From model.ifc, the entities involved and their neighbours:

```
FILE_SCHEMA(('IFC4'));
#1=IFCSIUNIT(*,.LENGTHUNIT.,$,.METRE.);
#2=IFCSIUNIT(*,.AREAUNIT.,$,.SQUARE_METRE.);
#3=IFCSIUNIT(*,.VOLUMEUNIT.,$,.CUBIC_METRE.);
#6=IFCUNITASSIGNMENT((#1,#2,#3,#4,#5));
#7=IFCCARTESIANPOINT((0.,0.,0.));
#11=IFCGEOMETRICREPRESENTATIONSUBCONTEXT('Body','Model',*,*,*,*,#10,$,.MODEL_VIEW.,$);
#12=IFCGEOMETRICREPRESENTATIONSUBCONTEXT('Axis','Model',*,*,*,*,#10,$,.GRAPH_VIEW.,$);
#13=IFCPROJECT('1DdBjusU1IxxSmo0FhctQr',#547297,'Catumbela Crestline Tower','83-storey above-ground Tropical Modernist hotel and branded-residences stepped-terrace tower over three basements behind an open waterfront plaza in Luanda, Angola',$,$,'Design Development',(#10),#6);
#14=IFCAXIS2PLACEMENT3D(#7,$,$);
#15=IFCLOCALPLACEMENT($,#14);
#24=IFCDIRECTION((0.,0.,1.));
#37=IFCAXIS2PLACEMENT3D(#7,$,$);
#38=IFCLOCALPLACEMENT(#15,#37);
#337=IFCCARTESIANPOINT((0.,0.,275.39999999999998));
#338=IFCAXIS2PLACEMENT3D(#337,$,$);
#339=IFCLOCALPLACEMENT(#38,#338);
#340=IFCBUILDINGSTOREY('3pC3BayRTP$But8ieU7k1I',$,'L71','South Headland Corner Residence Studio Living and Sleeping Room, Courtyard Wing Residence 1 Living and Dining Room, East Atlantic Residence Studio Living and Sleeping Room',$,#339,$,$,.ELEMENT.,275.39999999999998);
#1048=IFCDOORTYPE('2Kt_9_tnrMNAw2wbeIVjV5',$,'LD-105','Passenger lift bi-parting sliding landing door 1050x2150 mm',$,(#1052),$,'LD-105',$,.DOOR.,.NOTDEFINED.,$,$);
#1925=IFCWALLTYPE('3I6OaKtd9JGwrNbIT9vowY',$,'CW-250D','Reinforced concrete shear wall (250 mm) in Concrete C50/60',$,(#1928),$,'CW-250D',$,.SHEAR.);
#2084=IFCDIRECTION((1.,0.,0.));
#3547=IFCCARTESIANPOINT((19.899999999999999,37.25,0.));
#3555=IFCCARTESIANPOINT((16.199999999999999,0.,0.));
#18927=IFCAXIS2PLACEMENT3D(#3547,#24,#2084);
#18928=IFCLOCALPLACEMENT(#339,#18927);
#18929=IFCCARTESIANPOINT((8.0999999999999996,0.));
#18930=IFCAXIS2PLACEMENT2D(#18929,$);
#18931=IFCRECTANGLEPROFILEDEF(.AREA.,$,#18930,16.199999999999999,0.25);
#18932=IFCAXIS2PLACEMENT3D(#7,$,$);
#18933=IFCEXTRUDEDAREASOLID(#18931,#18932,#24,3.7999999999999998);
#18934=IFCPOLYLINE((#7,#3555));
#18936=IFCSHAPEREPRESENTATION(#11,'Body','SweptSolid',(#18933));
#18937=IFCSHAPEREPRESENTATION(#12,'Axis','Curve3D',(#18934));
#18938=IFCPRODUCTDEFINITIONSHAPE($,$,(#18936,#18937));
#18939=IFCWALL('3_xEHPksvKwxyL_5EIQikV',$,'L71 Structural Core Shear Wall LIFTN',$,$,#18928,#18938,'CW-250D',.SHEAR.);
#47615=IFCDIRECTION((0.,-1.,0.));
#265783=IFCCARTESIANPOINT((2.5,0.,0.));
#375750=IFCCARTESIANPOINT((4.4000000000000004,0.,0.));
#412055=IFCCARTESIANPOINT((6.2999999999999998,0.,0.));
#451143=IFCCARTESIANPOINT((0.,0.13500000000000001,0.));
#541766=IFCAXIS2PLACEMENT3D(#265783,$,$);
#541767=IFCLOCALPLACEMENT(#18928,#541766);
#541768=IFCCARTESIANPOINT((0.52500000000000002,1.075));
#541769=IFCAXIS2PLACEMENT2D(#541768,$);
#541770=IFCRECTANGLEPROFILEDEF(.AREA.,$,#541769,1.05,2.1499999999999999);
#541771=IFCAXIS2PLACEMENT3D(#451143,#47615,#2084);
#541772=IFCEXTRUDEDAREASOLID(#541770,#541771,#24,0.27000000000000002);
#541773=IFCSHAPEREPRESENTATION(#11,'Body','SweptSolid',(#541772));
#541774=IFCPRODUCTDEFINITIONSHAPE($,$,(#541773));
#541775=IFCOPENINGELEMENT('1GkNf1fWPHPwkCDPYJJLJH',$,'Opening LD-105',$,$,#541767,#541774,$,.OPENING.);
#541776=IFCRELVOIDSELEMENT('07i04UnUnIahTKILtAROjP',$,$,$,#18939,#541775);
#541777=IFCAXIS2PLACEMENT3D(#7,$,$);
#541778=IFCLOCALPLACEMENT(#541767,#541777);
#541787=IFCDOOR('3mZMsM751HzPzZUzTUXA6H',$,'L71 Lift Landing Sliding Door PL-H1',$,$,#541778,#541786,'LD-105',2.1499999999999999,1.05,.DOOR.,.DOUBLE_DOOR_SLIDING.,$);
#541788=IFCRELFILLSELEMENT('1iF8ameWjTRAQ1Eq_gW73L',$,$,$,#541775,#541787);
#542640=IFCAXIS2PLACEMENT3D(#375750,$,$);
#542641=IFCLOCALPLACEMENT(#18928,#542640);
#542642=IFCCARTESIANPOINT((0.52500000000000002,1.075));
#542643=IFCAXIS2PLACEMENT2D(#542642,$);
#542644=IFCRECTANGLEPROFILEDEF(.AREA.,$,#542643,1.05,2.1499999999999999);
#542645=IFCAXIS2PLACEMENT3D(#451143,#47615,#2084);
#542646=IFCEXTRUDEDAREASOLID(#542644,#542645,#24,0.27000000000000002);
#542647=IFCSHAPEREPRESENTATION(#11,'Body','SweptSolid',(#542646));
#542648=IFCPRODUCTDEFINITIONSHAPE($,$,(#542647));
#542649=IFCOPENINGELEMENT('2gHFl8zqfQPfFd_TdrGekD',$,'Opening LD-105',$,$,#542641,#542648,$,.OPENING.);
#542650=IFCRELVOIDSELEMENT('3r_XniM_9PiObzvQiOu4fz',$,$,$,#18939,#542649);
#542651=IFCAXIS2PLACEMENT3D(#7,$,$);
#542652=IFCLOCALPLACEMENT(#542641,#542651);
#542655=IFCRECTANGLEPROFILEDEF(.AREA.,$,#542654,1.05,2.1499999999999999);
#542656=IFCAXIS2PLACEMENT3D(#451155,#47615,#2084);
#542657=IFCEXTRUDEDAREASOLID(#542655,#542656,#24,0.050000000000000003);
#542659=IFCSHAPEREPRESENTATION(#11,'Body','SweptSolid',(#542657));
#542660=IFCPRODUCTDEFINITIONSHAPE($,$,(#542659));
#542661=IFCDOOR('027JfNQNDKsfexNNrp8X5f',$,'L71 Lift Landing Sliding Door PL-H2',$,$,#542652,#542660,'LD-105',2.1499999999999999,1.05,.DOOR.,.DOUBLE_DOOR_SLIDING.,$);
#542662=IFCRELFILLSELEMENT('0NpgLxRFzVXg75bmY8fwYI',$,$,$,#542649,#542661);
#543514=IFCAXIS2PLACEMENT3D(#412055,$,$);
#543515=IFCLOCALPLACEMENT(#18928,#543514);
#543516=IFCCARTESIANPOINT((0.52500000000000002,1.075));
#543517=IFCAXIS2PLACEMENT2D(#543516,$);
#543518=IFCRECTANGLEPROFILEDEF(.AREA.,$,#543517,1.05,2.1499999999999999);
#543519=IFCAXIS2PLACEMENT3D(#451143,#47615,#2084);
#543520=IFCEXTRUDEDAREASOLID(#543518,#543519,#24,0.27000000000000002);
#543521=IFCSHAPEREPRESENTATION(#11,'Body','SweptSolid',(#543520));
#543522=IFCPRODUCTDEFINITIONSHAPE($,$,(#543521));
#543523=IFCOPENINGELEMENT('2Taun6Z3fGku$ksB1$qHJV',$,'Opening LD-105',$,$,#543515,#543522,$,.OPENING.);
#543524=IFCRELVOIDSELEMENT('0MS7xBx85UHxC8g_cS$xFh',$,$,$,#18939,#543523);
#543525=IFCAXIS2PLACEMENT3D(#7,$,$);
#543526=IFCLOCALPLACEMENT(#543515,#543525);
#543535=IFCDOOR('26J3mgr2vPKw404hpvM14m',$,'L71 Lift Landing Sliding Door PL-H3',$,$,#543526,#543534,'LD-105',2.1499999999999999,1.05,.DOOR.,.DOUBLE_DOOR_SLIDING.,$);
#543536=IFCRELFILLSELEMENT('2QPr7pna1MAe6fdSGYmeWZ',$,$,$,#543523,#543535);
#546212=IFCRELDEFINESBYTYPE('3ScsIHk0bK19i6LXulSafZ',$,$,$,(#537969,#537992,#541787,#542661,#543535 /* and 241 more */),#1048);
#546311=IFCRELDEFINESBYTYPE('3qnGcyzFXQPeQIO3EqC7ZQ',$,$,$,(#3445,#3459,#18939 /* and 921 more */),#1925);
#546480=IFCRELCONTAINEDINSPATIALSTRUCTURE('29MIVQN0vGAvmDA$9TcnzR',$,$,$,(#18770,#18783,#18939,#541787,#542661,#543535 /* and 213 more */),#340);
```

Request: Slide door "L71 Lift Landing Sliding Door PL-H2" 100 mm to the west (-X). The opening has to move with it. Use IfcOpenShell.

```python
import ifcopenshell
import ifcopenshell.api.geometry
import ifcopenshell.util.placement
import ifcopenshell.util.unit

model = ifcopenshell.open("model.ifc")
unit_scale = ifcopenshell.util.unit.calculate_unit_scale(model)

door = model.by_guid("027JfNQNDKsfexNNrp8X5f")
opening = door.FillsVoids[0].RelatingOpeningElement
wall = opening.VoidsElements[0].RelatingBuildingElement

wall_matrix = ifcopenshell.util.placement.get_local_placement(wall.ObjectPlacement)
shift = wall_matrix[:3, 0] * -0.1 / unit_scale
before = ifcopenshell.util.placement.get_local_placement(door.ObjectPlacement)[:3, 3].copy()

# The door is placed relative to its opening, so it follows when the opening moves.
matrix = ifcopenshell.util.placement.get_local_placement(opening.ObjectPlacement)
matrix[:3, 3] += shift
ifcopenshell.api.geometry.edit_object_placement(
    model, product=opening, matrix=matrix, is_si=False, should_transform_children=True
)

after = ifcopenshell.util.placement.get_local_placement(door.ObjectPlacement)[:3, 3]
print("door moved by", (after - before).round(3) + 0.0)

model.write("model_v2.ifc")
```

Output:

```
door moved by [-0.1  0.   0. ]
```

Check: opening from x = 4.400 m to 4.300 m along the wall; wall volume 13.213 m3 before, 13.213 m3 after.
